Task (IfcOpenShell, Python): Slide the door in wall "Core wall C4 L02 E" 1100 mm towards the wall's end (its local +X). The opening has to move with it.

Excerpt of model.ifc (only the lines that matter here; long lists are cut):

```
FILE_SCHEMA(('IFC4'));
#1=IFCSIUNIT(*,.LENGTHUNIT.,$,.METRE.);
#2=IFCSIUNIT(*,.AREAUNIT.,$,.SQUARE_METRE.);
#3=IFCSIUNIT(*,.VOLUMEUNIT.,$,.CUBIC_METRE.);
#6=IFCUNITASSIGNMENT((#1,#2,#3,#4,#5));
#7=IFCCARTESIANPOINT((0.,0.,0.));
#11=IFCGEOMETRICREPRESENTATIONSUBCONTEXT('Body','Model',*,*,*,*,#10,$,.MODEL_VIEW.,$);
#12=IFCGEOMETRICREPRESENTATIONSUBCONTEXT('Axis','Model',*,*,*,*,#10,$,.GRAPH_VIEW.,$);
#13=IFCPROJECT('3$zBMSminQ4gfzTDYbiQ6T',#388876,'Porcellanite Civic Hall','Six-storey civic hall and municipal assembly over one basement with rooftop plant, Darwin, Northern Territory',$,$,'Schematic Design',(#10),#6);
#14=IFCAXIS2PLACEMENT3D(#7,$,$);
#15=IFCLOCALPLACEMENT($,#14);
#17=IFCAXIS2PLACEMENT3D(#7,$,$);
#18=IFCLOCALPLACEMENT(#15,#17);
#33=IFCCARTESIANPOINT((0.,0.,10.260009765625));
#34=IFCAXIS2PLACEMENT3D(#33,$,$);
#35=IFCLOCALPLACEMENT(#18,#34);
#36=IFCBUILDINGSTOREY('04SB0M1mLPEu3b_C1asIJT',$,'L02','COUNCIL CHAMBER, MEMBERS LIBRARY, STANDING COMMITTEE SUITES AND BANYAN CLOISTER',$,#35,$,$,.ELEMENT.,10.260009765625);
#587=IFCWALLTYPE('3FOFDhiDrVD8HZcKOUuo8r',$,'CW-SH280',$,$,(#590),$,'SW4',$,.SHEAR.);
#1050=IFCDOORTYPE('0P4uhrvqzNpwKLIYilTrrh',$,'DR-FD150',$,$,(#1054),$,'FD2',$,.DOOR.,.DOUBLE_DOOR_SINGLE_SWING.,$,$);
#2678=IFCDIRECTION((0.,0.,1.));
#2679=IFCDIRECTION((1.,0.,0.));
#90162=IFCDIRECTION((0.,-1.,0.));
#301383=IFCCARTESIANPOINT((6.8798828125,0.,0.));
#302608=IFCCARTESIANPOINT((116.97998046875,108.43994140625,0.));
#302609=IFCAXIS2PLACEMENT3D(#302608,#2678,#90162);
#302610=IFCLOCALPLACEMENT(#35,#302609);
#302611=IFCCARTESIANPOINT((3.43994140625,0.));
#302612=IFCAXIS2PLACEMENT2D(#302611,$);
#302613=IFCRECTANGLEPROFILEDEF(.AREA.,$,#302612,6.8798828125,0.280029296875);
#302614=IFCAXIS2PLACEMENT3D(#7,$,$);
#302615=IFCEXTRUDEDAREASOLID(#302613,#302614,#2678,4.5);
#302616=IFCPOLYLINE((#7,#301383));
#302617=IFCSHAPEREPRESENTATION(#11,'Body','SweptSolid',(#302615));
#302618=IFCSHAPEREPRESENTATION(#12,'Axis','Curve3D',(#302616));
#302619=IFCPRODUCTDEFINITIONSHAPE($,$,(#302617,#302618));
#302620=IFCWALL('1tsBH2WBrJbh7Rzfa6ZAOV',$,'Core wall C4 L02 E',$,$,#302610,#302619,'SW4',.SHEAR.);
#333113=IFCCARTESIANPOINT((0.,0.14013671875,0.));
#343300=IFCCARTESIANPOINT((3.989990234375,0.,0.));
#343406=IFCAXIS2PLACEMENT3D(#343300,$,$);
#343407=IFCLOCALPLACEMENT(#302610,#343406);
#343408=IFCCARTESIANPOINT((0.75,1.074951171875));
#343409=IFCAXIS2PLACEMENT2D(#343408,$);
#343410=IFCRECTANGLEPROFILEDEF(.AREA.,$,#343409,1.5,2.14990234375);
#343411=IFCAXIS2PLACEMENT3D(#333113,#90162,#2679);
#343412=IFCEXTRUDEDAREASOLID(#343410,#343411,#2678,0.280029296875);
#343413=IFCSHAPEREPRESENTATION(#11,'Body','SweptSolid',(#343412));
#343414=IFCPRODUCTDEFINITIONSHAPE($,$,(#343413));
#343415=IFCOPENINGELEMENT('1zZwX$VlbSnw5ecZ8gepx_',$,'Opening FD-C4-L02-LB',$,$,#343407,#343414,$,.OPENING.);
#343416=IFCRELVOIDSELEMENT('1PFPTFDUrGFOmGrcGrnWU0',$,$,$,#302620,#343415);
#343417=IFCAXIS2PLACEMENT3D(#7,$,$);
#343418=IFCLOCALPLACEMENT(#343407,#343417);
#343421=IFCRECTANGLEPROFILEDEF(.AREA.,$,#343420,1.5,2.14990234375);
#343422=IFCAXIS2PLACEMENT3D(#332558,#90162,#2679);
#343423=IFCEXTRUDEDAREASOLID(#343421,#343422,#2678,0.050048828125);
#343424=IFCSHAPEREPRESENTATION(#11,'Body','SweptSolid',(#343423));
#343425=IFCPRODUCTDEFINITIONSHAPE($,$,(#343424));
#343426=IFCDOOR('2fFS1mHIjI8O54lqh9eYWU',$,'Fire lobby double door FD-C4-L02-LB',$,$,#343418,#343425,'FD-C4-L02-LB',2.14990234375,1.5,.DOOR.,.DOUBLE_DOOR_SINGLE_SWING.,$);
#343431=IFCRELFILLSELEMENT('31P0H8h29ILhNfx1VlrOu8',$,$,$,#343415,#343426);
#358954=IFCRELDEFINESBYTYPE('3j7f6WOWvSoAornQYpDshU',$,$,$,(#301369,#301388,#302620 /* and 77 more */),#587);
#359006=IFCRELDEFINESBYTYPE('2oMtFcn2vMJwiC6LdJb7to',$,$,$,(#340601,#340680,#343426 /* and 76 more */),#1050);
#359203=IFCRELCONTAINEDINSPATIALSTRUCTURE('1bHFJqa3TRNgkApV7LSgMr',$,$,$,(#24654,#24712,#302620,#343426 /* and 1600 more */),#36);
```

```python
import ifcopenshell
import ifcopenshell.api.geometry
import ifcopenshell.util.placement
import ifcopenshell.util.unit

model = ifcopenshell.open("model.ifc")
unit_scale = ifcopenshell.util.unit.calculate_unit_scale(model)

door = model.by_guid("2fFS1mHIjI8O54lqh9eYWU")
opening = door.FillsVoids[0].RelatingOpeningElement
wall = opening.VoidsElements[0].RelatingBuildingElement

wall_matrix = ifcopenshell.util.placement.get_local_placement(wall.ObjectPlacement)
shift = wall_matrix[:3, 0] * 1.1 / unit_scale
before = ifcopenshell.util.placement.get_local_placement(door.ObjectPlacement)[:3, 3].copy()

# The door is placed relative to its opening, so it follows when the opening moves.
matrix = ifcopenshell.util.placement.get_local_placement(opening.ObjectPlacement)
matrix[:3, 3] += shift
ifcopenshell.api.geometry.edit_object_placement(
    model, product=opening, matrix=matrix, is_si=False, should_transform_children=True
)

after = ifcopenshell.util.placement.get_local_placement(door.ObjectPlacement)[:3, 3]
print("door moved by", (after - before).round(3) + 0.0)

model.write("model_rev.ifc")
```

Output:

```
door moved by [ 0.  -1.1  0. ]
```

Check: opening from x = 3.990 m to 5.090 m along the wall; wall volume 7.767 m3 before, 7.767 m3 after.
